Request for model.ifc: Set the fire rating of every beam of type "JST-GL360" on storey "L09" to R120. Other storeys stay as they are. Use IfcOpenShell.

First a look at what the model holds.

```python
import ifcopenshell
import ifcopenshell.util.element

model = ifcopenshell.open("model.ifc")
print(model.schema)
storey = next(s for s in model.by_type("IfcBuildingStorey") if s.Name == "L09")
beams = [e for e in ifcopenshell.util.element.get_decomposition(storey) if e.is_a("IfcBeam")]
seen = {}
for e in beams:
    element_type = ifcopenshell.util.element.get_type(e)
    key = (element_type.Name if element_type != e and element_type else None, ifcopenshell.util.element.get_pset(e, "Pset_BeamCommon", "FireRating"))
    seen[key] = seen.get(key, 0) + 1
for (name, value), count in sorted(seen.items(), key=str):
    print(count, "x", name, "|", value)
```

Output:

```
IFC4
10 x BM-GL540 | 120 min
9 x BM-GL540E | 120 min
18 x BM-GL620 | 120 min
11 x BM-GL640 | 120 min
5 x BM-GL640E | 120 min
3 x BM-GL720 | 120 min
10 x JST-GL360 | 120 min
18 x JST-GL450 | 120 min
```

```python
import ifcopenshell
import ifcopenshell.api.pset
import ifcopenshell.util.element

model = ifcopenshell.open("model.ifc")

storey = next(s for s in model.by_type("IfcBuildingStorey") if s.Name == "L09")
beams = [e for e in ifcopenshell.util.element.get_decomposition(storey) if e.is_a("IfcBeam")]

count = 0
for e in beams:
    element_type = ifcopenshell.util.element.get_type(e)
    if element_type in (None, e) or element_type.Name != "JST-GL360":
        continue
    # add_pset returns the element's existing set when there is one.
    pset = ifcopenshell.api.pset.add_pset(model, product=e, name="Pset_BeamCommon")
    ifcopenshell.api.pset.edit_pset(model, pset=pset, properties={"FireRating": "R120"})
    count += 1

print(count, "beams updated")

model.write("model_rev.ifc")
```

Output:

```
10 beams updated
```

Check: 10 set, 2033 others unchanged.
